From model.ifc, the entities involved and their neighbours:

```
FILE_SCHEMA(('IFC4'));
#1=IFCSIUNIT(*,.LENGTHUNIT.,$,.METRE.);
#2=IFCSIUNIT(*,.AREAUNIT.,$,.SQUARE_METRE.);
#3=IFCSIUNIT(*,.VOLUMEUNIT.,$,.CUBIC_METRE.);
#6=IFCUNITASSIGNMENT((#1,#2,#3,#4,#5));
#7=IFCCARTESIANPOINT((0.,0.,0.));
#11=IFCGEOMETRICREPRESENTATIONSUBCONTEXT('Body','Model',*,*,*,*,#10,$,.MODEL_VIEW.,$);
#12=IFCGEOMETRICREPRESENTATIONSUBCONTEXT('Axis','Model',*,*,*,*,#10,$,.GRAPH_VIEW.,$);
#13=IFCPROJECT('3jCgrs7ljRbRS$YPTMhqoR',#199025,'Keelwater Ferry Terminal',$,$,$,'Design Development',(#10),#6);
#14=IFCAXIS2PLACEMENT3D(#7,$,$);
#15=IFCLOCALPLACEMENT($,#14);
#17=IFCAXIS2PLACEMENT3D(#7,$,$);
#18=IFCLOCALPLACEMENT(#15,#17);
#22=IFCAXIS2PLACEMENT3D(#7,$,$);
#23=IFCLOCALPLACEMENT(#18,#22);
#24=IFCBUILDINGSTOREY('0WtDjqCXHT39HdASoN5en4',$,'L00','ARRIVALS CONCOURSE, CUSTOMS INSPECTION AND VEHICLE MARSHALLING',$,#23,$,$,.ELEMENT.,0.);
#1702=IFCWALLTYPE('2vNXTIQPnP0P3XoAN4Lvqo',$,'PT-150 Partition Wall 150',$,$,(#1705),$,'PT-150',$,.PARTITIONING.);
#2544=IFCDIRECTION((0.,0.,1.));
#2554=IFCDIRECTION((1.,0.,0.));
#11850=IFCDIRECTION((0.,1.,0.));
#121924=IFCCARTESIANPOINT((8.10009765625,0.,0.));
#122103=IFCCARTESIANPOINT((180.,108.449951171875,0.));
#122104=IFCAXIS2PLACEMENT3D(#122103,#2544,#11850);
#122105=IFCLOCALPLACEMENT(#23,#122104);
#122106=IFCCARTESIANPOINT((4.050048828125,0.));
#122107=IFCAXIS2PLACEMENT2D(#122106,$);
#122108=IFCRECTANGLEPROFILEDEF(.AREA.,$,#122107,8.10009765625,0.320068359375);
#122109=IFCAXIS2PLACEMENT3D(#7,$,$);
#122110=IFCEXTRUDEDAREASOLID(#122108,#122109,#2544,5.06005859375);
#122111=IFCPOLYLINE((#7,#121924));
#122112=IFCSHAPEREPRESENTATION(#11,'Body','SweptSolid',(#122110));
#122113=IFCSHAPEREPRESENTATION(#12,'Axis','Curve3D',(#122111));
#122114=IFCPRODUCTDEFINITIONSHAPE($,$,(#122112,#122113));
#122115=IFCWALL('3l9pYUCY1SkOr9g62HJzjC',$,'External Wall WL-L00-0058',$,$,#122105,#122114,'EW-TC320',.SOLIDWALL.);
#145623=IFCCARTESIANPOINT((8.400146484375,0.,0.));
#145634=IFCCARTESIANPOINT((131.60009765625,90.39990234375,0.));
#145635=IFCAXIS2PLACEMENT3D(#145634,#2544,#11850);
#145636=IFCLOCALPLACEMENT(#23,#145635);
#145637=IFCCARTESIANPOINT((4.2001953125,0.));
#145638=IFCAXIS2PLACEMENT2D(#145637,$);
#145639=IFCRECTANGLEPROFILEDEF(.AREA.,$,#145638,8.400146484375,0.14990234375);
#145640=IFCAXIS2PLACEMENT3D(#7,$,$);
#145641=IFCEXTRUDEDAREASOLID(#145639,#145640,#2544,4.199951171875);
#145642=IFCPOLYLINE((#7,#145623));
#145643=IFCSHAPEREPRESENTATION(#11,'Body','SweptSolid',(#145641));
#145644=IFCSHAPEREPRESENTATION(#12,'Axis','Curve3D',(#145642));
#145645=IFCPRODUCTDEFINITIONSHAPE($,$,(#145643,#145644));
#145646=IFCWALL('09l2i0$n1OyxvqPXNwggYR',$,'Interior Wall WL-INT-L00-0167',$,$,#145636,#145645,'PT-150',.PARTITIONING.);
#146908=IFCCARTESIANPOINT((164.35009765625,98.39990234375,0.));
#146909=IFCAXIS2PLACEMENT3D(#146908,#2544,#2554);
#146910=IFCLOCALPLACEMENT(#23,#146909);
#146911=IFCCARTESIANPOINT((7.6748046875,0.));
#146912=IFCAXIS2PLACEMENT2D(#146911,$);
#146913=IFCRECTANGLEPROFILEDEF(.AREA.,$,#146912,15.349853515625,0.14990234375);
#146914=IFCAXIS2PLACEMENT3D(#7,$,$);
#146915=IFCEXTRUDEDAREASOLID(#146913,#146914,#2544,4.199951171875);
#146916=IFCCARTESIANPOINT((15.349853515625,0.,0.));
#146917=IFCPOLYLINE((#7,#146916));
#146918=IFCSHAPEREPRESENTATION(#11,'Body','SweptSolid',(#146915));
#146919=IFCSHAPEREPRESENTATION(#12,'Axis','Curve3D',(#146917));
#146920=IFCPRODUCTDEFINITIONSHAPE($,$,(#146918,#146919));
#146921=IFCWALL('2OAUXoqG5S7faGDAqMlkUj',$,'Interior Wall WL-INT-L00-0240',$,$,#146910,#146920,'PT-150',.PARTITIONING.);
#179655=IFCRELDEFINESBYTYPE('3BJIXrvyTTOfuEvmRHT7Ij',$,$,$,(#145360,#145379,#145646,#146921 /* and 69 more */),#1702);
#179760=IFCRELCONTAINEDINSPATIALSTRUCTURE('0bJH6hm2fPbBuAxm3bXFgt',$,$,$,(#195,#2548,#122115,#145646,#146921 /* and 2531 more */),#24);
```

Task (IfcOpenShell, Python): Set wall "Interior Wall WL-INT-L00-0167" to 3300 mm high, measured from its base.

```python
import ifcopenshell
import ifcopenshell.geom
import ifcopenshell.util.representation
import ifcopenshell.util.shape
import ifcopenshell.util.unit

model = ifcopenshell.open("model.ifc")
unit_scale = ifcopenshell.util.unit.calculate_unit_scale(model)
settings = ifcopenshell.geom.settings()


def volume(element):
    """Net volume in cubic metres, openings subtracted."""
    shape = ifcopenshell.geom.create_shape(settings, element)
    return ifcopenshell.util.shape.get_volume(shape.geometry)


wall = model.by_guid("09l2i0$n1OyxvqPXNwggYR")
before = volume(wall)

body = ifcopenshell.util.representation.get_representation(wall, "Model", "Body")
solid = body.Items[0]
old_height = solid.Depth
solid.Depth = 3.3 / unit_scale
after = volume(wall)

print(f"height {old_height:g} -> {solid.Depth:g}, volume {before:.3f} -> {after:.3f} m3")

model.write("model-out.ifc")
```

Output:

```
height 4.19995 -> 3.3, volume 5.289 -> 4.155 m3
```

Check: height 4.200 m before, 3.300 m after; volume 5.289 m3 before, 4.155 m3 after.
